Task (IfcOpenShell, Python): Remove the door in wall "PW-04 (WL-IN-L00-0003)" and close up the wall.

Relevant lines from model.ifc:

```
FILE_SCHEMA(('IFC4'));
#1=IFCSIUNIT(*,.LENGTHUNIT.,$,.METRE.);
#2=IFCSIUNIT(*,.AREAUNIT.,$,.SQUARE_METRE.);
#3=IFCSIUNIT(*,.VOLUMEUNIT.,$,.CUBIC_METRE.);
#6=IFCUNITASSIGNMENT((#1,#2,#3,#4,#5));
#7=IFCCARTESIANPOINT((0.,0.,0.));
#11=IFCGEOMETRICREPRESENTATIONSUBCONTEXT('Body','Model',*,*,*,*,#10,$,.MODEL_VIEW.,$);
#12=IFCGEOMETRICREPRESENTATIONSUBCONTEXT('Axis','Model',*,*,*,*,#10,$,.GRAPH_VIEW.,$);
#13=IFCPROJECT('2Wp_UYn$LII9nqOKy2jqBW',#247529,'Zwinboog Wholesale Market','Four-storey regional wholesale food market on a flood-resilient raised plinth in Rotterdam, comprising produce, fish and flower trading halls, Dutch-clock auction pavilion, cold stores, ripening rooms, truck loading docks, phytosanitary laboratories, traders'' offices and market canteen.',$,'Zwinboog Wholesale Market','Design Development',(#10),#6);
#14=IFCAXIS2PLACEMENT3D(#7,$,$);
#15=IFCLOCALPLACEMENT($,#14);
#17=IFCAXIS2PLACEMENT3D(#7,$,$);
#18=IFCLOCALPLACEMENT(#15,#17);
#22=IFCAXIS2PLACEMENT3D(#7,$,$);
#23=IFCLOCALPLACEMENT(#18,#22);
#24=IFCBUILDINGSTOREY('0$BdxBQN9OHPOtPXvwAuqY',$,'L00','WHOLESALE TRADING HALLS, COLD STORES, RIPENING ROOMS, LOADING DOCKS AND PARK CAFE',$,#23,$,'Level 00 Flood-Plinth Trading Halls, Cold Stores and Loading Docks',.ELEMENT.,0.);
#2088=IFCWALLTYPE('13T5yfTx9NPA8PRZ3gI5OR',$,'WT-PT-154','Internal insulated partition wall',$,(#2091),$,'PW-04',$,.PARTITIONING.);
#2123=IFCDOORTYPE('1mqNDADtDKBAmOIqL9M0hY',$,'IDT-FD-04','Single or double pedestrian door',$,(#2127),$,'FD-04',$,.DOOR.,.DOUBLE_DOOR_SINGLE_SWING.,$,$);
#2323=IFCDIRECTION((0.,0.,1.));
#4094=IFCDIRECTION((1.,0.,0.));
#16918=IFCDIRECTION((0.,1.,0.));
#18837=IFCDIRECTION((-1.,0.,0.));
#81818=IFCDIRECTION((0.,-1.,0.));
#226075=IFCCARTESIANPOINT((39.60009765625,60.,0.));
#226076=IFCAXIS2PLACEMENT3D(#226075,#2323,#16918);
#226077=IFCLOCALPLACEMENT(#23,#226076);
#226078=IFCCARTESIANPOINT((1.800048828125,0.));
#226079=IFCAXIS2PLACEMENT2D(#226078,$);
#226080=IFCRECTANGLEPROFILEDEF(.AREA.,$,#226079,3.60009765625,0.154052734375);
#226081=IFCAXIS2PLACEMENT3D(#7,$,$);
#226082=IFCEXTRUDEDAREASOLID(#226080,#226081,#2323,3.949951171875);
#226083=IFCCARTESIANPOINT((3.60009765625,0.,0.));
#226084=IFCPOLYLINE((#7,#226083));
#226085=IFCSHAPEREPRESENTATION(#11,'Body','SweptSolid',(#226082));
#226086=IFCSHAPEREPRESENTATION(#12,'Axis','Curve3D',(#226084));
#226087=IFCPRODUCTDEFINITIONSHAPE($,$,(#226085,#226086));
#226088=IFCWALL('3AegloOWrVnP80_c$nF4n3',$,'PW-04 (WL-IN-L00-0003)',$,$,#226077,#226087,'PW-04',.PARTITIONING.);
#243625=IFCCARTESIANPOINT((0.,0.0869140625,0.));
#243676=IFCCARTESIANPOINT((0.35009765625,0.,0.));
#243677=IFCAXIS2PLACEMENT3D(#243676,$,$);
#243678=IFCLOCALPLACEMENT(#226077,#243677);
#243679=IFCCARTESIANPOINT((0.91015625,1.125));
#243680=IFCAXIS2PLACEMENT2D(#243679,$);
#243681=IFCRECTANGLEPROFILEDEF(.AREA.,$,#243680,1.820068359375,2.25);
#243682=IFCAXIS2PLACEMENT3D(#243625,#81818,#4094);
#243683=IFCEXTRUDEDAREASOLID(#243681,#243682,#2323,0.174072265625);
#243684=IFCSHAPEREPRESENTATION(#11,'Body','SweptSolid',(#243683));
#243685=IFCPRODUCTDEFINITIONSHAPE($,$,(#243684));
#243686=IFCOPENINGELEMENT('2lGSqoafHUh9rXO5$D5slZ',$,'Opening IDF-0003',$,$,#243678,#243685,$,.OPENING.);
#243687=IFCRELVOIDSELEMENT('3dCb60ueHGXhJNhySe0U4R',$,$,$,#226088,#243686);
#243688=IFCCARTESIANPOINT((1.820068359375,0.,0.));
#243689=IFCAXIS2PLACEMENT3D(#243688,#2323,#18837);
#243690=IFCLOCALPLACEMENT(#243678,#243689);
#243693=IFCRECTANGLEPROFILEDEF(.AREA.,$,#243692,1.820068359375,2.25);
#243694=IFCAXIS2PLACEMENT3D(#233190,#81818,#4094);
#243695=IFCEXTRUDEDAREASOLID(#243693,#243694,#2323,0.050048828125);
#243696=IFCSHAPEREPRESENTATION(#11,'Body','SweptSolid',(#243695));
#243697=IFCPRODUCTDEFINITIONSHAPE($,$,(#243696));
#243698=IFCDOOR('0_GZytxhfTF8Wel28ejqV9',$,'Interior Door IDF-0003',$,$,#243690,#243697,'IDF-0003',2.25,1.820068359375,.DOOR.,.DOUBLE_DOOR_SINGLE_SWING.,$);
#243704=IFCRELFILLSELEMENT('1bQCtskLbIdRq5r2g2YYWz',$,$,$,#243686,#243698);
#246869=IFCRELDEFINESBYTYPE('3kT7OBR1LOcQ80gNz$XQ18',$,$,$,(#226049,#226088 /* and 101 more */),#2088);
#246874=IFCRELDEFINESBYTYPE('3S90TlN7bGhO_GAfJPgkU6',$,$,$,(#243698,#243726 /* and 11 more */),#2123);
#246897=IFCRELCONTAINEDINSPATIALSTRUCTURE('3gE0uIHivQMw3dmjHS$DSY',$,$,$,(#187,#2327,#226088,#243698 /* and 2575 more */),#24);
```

```python
import ifcopenshell
import ifcopenshell.api.feature
import ifcopenshell.api.root
import ifcopenshell.geom
import ifcopenshell.util.shape

model = ifcopenshell.open("model.ifc")
settings = ifcopenshell.geom.settings()


def volume(element):
    """Net volume in cubic metres, openings subtracted."""
    shape = ifcopenshell.geom.create_shape(settings, element)
    return ifcopenshell.util.shape.get_volume(shape.geometry)


door = model.by_id(243698)
opening = door.FillsVoids[0].RelatingOpeningElement
wall = opening.VoidsElements[0].RelatingBuildingElement
before = volume(wall)

ifcopenshell.api.root.remove_product(model, product=door)
ifcopenshell.api.feature.remove_feature(model, feature=opening)

after = volume(wall)

print(f"wall volume {before:.3f} -> {after:.3f} m3")

model.write("model_edited.ifc")
```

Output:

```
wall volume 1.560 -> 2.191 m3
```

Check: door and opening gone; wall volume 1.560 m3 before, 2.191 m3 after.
